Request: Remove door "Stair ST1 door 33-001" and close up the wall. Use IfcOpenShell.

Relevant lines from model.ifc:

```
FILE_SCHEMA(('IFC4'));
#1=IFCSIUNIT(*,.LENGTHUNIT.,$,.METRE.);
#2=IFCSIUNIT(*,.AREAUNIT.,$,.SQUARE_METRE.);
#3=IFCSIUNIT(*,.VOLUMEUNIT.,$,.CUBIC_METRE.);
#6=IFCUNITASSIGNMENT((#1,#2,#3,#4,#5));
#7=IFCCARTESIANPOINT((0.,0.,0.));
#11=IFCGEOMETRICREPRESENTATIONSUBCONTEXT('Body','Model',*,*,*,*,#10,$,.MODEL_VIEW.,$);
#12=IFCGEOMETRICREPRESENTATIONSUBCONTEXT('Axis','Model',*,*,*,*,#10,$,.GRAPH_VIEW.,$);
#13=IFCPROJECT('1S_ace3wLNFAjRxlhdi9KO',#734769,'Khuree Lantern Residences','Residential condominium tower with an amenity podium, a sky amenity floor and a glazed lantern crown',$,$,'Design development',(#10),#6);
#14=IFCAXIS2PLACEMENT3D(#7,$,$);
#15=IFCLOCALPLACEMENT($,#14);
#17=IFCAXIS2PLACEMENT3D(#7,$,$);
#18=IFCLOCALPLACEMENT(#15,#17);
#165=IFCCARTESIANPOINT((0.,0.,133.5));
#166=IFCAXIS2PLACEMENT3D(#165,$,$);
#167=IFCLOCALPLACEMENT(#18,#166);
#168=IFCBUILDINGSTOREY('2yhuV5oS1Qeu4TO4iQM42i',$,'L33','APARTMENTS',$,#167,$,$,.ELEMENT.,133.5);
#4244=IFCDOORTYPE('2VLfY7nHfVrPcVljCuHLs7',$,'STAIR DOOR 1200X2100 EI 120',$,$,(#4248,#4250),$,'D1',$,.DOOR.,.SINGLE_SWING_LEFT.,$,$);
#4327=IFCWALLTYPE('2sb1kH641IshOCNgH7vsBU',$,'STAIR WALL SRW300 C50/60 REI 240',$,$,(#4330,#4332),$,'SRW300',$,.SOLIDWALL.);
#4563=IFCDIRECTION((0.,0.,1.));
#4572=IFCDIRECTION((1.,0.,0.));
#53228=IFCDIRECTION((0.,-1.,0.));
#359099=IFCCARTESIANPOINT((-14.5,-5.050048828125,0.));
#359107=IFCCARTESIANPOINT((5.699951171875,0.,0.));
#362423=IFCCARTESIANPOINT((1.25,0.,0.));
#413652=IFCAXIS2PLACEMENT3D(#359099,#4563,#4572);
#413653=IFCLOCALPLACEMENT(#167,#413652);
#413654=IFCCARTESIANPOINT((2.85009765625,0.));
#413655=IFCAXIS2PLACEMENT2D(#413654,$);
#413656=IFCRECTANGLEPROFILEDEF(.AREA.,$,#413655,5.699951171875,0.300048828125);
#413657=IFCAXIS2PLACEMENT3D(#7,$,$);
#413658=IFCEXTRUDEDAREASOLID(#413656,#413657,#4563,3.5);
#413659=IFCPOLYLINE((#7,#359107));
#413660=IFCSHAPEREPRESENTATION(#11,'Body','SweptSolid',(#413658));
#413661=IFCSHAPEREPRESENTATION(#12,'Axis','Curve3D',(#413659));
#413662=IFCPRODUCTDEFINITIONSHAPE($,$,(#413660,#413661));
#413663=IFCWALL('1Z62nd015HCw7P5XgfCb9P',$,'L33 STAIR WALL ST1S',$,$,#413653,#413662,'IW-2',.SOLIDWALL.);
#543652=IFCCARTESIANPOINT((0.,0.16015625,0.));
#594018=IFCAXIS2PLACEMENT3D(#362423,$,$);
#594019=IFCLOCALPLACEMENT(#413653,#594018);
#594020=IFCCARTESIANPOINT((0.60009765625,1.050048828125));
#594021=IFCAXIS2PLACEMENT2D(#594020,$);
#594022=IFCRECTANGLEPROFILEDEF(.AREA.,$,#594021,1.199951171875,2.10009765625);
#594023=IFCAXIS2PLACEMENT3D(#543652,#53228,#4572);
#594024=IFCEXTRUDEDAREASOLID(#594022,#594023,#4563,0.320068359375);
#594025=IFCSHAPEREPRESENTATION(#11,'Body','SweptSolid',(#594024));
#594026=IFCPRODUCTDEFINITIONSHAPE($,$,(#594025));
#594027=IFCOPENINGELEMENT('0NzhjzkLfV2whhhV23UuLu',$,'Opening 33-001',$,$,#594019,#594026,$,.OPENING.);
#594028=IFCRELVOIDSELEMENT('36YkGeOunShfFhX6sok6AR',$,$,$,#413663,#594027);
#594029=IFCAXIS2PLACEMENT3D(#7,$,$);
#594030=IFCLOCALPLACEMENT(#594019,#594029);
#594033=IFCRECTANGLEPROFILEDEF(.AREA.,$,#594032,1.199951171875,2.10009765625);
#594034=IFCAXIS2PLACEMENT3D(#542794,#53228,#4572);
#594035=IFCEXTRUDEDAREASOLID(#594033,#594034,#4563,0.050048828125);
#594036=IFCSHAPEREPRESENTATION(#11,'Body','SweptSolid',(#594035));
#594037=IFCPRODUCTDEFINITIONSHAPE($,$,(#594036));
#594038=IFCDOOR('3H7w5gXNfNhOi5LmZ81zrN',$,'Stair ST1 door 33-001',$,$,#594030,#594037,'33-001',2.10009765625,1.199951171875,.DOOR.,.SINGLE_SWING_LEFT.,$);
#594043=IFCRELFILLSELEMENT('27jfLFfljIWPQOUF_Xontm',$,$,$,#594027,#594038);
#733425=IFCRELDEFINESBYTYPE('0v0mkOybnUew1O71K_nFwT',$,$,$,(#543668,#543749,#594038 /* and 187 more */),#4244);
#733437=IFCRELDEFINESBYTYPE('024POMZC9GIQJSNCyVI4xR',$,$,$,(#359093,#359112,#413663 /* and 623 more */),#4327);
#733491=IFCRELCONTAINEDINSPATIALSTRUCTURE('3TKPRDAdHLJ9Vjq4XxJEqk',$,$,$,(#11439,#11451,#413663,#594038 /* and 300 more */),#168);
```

```python
import ifcopenshell
import ifcopenshell.api.feature
import ifcopenshell.api.root
import ifcopenshell.geom
import ifcopenshell.util.shape

model = ifcopenshell.open("model.ifc")
settings = ifcopenshell.geom.settings()


def volume(element):
    """Net volume in cubic metres, openings subtracted."""
    shape = ifcopenshell.geom.create_shape(settings, element)
    return ifcopenshell.util.shape.get_volume(shape.geometry)


door = model.by_guid("3H7w5gXNfNhOi5LmZ81zrN")
opening = door.FillsVoids[0].RelatingOpeningElement
wall = opening.VoidsElements[0].RelatingBuildingElement
before = volume(wall)

ifcopenshell.api.root.remove_product(model, product=door)
ifcopenshell.api.feature.remove_feature(model, feature=opening)

after = volume(wall)

print(f"wall volume {before:.3f} -> {after:.3f} m3")

model.write("model_v2.ifc")
```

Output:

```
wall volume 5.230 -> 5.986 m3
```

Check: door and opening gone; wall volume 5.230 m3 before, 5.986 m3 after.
